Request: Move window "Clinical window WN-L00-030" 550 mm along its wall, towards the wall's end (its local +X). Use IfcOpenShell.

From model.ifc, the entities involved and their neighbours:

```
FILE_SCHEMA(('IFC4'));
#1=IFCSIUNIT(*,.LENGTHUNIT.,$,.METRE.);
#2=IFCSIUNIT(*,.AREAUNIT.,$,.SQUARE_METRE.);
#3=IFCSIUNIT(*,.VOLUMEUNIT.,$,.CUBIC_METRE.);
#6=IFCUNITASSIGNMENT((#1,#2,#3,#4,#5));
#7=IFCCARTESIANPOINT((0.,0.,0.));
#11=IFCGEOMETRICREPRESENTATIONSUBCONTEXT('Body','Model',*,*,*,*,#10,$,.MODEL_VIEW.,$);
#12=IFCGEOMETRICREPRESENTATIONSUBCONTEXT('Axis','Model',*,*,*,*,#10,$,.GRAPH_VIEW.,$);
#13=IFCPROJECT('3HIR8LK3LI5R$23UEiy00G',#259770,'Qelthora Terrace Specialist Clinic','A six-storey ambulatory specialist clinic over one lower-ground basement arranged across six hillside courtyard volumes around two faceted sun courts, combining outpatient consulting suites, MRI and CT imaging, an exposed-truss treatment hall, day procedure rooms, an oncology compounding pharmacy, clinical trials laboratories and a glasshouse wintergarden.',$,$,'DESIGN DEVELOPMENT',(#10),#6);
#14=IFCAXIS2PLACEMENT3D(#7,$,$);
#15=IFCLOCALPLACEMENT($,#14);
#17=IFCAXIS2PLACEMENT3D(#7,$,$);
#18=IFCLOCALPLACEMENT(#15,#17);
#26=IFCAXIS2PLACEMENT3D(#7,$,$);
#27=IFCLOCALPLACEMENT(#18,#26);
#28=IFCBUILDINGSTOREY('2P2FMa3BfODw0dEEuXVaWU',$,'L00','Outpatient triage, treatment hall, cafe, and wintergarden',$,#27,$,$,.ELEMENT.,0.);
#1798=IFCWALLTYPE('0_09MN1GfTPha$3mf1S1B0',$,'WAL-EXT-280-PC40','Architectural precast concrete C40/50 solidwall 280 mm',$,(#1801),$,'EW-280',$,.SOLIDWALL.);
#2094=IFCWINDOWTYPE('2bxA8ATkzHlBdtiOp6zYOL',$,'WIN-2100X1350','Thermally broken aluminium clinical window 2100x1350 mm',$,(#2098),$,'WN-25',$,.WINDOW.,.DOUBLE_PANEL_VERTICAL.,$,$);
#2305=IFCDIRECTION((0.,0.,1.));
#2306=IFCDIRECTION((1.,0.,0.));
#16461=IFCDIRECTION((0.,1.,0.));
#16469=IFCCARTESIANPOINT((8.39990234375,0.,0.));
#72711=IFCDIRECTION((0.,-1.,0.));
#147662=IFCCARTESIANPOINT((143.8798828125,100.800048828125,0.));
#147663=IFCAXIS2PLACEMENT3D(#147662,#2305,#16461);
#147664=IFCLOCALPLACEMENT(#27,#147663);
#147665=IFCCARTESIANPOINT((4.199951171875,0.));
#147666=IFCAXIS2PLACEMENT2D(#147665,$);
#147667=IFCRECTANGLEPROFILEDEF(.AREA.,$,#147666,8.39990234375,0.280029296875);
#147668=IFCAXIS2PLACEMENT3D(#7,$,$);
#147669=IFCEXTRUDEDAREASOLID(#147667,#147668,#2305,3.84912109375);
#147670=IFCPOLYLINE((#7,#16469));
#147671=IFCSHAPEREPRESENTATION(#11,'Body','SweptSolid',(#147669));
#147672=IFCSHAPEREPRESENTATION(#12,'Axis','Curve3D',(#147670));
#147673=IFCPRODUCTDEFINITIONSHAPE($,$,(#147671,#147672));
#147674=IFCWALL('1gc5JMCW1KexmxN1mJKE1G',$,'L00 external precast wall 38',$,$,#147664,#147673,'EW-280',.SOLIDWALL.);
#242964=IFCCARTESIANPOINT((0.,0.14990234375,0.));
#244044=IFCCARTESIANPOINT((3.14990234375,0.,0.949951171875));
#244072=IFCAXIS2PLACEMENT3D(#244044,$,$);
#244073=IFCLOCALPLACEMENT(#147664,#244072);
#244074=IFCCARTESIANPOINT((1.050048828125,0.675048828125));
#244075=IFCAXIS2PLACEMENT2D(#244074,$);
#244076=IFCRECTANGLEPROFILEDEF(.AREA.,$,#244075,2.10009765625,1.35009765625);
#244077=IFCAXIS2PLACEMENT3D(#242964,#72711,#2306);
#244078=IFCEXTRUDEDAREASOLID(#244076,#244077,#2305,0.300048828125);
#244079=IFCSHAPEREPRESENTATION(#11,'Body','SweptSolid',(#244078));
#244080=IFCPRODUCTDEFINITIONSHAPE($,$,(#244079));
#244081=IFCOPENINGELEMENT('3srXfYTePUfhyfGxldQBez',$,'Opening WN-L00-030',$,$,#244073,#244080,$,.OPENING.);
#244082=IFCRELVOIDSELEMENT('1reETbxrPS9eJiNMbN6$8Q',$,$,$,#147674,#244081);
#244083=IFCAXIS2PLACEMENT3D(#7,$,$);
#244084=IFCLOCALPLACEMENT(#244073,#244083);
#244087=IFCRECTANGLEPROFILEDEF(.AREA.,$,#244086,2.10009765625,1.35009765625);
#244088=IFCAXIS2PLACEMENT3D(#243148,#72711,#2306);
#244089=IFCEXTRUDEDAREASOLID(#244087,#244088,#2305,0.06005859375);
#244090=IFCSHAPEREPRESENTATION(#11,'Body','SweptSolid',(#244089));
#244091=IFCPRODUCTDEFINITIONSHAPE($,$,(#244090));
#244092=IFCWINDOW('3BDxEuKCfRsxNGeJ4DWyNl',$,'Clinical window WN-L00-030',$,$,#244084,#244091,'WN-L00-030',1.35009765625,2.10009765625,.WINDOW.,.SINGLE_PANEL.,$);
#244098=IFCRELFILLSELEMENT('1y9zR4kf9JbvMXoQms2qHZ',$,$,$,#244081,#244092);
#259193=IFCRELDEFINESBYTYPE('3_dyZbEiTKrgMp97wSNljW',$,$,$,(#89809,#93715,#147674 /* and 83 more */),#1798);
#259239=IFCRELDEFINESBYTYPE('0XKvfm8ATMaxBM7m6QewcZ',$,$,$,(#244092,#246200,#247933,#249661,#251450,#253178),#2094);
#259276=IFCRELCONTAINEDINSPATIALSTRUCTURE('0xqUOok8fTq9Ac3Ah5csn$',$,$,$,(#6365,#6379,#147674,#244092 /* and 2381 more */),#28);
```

```python
import ifcopenshell
import ifcopenshell.api.geometry
import ifcopenshell.util.placement
import ifcopenshell.util.unit

model = ifcopenshell.open("model.ifc")
unit_scale = ifcopenshell.util.unit.calculate_unit_scale(model)

window = model.by_id(244092)
opening = window.FillsVoids[0].RelatingOpeningElement
wall = opening.VoidsElements[0].RelatingBuildingElement

wall_matrix = ifcopenshell.util.placement.get_local_placement(wall.ObjectPlacement)
shift = wall_matrix[:3, 0] * 0.55 / unit_scale
before = ifcopenshell.util.placement.get_local_placement(window.ObjectPlacement)[:3, 3].copy()

# The window is placed relative to its opening, so it follows when the opening moves.
matrix = ifcopenshell.util.placement.get_local_placement(opening.ObjectPlacement)
matrix[:3, 3] += shift
ifcopenshell.api.geometry.edit_object_placement(
    model, product=opening, matrix=matrix, is_si=False, should_transform_children=True
)

after = ifcopenshell.util.placement.get_local_placement(window.ObjectPlacement)[:3, 3]
print("window moved by", (after - before).round(3) + 0.0)

model.write("model_v2.ifc")
```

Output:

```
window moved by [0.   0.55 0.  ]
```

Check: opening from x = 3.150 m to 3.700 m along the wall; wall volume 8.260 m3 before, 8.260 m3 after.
